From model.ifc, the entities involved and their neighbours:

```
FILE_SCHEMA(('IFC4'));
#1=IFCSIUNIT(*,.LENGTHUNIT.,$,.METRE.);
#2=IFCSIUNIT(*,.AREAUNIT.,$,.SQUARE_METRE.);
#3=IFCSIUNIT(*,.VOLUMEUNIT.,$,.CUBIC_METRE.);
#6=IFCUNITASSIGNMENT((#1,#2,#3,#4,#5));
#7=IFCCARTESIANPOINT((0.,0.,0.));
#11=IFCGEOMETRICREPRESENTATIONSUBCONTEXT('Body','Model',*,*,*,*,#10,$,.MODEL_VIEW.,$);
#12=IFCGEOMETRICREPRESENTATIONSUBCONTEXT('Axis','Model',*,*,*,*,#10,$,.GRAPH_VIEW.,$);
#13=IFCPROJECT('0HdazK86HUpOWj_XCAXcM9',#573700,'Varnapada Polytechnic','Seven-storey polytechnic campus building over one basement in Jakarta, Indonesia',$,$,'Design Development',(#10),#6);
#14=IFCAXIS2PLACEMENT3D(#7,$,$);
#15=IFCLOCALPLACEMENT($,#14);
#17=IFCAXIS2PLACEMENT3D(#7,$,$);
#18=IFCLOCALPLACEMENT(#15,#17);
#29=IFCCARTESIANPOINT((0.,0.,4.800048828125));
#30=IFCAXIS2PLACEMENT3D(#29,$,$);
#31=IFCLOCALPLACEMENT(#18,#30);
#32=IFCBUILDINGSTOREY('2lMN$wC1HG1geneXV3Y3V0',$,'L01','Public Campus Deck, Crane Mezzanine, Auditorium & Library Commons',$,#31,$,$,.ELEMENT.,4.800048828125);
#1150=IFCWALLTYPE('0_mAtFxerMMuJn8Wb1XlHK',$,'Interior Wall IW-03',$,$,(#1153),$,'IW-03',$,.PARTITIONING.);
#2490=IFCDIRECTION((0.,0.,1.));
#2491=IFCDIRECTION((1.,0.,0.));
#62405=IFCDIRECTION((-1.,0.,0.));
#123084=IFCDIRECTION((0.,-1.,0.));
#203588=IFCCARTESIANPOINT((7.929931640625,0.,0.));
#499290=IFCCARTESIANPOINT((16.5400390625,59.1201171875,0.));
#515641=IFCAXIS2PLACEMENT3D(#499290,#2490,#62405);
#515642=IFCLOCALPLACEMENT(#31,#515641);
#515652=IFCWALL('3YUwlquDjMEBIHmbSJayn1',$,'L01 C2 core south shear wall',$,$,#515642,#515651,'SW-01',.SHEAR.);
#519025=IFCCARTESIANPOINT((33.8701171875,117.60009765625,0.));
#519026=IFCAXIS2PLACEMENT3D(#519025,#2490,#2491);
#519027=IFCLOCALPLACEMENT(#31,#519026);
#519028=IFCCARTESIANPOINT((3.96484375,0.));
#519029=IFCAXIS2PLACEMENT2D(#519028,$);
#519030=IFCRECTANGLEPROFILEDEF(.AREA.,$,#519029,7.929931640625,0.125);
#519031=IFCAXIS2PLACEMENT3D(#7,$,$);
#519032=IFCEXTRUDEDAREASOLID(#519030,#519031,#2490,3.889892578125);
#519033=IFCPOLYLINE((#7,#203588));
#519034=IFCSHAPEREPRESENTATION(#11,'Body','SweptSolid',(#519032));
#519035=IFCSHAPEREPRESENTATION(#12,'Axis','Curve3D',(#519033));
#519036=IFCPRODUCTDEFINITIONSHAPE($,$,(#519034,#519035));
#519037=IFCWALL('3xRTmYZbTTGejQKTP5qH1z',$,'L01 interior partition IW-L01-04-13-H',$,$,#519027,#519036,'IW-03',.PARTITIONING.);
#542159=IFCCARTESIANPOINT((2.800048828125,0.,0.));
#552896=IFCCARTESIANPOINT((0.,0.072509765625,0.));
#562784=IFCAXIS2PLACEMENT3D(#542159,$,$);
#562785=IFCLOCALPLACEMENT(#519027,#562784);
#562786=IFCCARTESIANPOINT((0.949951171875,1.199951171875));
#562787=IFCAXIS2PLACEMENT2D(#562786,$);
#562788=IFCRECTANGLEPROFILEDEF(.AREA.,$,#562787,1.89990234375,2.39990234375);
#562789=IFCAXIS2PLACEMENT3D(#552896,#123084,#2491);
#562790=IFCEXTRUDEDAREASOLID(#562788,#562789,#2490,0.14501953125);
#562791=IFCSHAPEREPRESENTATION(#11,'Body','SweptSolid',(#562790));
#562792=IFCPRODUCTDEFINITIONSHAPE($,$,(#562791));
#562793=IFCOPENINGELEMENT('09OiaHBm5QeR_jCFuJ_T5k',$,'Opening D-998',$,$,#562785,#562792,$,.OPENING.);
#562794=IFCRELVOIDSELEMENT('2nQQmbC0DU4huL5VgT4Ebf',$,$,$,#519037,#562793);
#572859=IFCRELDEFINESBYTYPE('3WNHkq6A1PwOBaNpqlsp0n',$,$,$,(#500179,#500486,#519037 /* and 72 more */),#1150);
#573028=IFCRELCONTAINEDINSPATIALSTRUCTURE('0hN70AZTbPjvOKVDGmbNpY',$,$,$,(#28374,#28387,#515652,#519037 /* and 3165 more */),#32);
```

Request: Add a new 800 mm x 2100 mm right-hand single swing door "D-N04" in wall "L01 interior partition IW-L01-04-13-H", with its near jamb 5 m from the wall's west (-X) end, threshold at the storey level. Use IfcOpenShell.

```python
import numpy as np
import ifcopenshell
import ifcopenshell.api.feature
import ifcopenshell.api.geometry
import ifcopenshell.api.root
import ifcopenshell.api.spatial
import ifcopenshell.geom
import ifcopenshell.util.element
import ifcopenshell.util.placement
import ifcopenshell.util.representation
import ifcopenshell.util.shape
import ifcopenshell.util.unit

model = ifcopenshell.open("model.ifc")
unit_scale = ifcopenshell.util.unit.calculate_unit_scale(model)
settings = ifcopenshell.geom.settings()


def volume(element):
    """Net volume in cubic metres, openings subtracted."""
    shape = ifcopenshell.geom.create_shape(settings, element)
    return ifcopenshell.util.shape.get_volume(shape.geometry)


wall = model.by_id(519037)
storey = ifcopenshell.util.element.get_container(wall, ifc_class="IfcBuildingStorey")
context = ifcopenshell.util.representation.get_context(model, "Model", "Body", "MODEL_VIEW")
before = volume(wall)

width, height, from_end, sill = 0.8, 2.1, 5, 0.0  # metres

# The wall runs along its own X axis, and the end named is its -X end.
wall_shape = ifcopenshell.geom.create_shape(settings, wall)
x, y, z = ifcopenshell.util.shape.get_vertices(wall_shape.geometry).T
start = x.min() + from_end
face, thickness = float(y.min()), float(y.max() - y.min())
wall_matrix = ifcopenshell.util.placement.get_local_placement(wall.ObjectPlacement)
level = ifcopenshell.util.placement.get_local_placement(storey.ObjectPlacement)[2, 3]


def in_wall(x, y):
    """Placement at x, y metres in the wall's axes, at sill height."""
    matrix = wall_matrix.copy()
    matrix[:, 3] = wall_matrix @ np.array([x / unit_scale, y / unit_scale, 0.0, 1.0])
    matrix[2, 3] = level + sill / unit_scale
    return matrix


# Opening: a box that overshoots both wall faces by 50 mm.
opening = ifcopenshell.api.root.create_entity(model, ifc_class="IfcOpeningElement", predefined_type="OPENING")
box = ifcopenshell.api.geometry.add_wall_representation(
    model, context=context, length=width, height=height, thickness=thickness + 0.1
)
ifcopenshell.api.geometry.assign_representation(model, product=opening, representation=box)
ifcopenshell.api.geometry.edit_object_placement(model, product=opening, matrix=in_wall(start, face - 0.05), is_si=False)
ifcopenshell.api.feature.add_feature(model, feature=opening, element=wall)

door = ifcopenshell.api.root.create_entity(model, ifc_class="IfcDoor", name="D-N04", predefined_type="DOOR")
door.OverallWidth, door.OverallHeight = width / unit_scale, height / unit_scale
door.OperationType = "SINGLE_SWING_RIGHT"
body = ifcopenshell.api.geometry.add_door_representation(
    model,
    context=context,
    overall_width=door.OverallWidth,
    overall_height=door.OverallHeight,
    operation_type="SINGLE_SWING_RIGHT",
    lining_properties={"LiningDepth": thickness / unit_scale, "ThresholdDepth": thickness / unit_scale},
)
ifcopenshell.api.geometry.assign_representation(model, product=door, representation=body)
ifcopenshell.api.spatial.assign_container(model, products=[door], relating_structure=storey)
ifcopenshell.api.feature.add_filling(model, opening=opening, element=door)

# The lining spans the wall, so the door starts at the wall face.
ifcopenshell.api.geometry.edit_object_placement(model, product=door, matrix=in_wall(start, face), is_si=False)

after = volume(wall)

print(f"wall volume {before:.3f} -> {after:.3f} m3")

model.write("model-out.ifc")
```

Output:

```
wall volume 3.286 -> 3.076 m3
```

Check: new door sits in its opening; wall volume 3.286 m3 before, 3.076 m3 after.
